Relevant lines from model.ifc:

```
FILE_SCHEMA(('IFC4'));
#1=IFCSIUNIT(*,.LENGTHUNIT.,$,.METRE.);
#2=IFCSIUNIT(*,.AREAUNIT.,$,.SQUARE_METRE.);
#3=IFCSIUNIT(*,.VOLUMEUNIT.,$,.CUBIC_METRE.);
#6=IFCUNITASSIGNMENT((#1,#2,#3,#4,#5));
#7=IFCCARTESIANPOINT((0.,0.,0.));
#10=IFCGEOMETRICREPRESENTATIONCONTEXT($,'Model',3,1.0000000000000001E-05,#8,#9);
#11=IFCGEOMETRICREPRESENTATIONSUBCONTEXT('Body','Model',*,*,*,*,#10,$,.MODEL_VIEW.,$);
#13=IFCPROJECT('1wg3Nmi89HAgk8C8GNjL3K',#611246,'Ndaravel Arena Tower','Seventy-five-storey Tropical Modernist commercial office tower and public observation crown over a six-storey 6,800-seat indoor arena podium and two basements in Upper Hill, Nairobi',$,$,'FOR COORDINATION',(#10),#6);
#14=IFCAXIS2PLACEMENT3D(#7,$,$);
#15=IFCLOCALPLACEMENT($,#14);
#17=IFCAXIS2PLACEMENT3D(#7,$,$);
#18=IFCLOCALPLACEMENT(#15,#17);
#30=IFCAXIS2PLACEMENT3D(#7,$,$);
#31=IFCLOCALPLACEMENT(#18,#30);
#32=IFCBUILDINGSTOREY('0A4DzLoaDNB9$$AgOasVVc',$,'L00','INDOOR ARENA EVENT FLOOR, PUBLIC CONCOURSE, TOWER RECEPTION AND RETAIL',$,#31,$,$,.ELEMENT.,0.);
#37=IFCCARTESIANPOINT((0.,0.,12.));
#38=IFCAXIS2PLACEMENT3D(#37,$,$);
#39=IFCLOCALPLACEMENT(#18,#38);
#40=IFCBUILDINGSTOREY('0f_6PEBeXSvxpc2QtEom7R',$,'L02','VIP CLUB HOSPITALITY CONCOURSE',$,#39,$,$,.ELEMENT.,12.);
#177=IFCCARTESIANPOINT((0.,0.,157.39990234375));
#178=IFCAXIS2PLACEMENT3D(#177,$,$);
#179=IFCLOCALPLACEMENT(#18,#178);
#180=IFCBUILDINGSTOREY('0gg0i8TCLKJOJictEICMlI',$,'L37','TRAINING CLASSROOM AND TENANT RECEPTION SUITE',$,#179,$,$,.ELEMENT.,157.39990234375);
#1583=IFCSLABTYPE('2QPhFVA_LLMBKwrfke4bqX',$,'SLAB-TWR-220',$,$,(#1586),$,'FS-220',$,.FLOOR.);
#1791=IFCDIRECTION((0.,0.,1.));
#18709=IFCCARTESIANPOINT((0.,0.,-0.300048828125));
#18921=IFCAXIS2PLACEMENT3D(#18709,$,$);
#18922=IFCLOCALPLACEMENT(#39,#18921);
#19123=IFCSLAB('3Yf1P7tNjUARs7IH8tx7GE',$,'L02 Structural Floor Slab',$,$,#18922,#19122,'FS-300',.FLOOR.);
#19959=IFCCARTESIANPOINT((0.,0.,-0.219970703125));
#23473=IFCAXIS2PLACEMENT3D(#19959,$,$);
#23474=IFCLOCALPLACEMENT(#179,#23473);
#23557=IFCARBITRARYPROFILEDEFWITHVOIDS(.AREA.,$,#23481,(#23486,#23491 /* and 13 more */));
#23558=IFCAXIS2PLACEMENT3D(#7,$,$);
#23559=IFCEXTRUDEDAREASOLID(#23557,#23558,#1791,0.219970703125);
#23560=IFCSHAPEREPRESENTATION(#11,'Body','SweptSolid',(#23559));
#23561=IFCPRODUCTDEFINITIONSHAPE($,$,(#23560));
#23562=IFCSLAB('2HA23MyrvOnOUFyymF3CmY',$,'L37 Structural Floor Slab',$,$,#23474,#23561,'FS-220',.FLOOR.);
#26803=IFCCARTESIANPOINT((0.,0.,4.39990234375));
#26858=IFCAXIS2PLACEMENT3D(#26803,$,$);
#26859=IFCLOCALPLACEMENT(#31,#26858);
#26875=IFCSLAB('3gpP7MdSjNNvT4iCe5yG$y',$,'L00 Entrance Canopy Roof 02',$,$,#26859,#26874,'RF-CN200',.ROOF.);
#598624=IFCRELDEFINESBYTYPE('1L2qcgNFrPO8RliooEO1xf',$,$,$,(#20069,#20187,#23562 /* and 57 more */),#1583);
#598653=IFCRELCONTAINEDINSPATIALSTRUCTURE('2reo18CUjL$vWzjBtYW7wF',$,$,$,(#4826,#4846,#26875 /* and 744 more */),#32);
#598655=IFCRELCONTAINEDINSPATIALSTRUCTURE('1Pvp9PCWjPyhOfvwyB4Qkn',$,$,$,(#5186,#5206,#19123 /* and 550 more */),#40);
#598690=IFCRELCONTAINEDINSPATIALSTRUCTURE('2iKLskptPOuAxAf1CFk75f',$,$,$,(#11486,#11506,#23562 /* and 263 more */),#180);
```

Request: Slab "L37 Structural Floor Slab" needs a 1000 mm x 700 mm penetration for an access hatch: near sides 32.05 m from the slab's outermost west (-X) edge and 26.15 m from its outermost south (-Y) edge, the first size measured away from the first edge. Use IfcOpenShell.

```python
import numpy as np
import ifcopenshell
import ifcopenshell.api.feature
import ifcopenshell.api.geometry
import ifcopenshell.api.root
import ifcopenshell.geom
import ifcopenshell.util.placement
import ifcopenshell.util.representation
import ifcopenshell.util.shape
import ifcopenshell.util.unit

model = ifcopenshell.open("model.ifc")
unit_scale = ifcopenshell.util.unit.calculate_unit_scale(model)
settings = ifcopenshell.geom.settings()


def volume(element):
    """Net volume in cubic metres, openings subtracted."""
    shape = ifcopenshell.geom.create_shape(settings, element)
    return ifcopenshell.util.shape.get_volume(shape.geometry)


slab = model.by_id(23562)
before = volume(slab)

# Extent in the slab's own axes, in metres. The edges named are its -X and -Y sides.
slab_shape = ifcopenshell.geom.create_shape(settings, slab)
vertices = ifcopenshell.util.shape.get_vertices(slab_shape.geometry)
x_min, y_min, bottom = vertices.min(axis=0)
top = vertices[:, 2].max()

opening = ifcopenshell.api.root.create_entity(model, ifc_class="IfcOpeningElement", name="Access hatch opening", predefined_type="OPENING")
context = ifcopenshell.util.representation.get_context(model, "Model", "Body", "MODEL_VIEW")
width, depth = 1, 0.7
outline = [(0.0, 0.0), (width, 0.0), (width, depth), (0.0, depth), (0.0, 0.0)]
# Overshoot both faces by 50 mm so the cut is clean.
shape = ifcopenshell.api.geometry.add_slab_representation(
    model, context=context, depth=top - bottom + 0.1, polyline=outline
)
ifcopenshell.api.geometry.assign_representation(model, product=opening, representation=shape)

matrix = ifcopenshell.util.placement.get_local_placement(slab.ObjectPlacement)
matrix[:, 3] = matrix @ np.append(np.array([x_min + 32.05, y_min + 26.15, bottom - 0.05]) / unit_scale, 1.0)
ifcopenshell.api.geometry.edit_object_placement(model, product=opening, matrix=matrix, is_si=False)
ifcopenshell.api.feature.add_feature(model, feature=opening, element=slab)

after = volume(slab)

print(f"slab volume {before:.3f} -> {after:.3f} m3")

model.write("model_updated.ifc")
```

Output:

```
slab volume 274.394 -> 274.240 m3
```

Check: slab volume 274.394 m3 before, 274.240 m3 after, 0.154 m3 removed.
